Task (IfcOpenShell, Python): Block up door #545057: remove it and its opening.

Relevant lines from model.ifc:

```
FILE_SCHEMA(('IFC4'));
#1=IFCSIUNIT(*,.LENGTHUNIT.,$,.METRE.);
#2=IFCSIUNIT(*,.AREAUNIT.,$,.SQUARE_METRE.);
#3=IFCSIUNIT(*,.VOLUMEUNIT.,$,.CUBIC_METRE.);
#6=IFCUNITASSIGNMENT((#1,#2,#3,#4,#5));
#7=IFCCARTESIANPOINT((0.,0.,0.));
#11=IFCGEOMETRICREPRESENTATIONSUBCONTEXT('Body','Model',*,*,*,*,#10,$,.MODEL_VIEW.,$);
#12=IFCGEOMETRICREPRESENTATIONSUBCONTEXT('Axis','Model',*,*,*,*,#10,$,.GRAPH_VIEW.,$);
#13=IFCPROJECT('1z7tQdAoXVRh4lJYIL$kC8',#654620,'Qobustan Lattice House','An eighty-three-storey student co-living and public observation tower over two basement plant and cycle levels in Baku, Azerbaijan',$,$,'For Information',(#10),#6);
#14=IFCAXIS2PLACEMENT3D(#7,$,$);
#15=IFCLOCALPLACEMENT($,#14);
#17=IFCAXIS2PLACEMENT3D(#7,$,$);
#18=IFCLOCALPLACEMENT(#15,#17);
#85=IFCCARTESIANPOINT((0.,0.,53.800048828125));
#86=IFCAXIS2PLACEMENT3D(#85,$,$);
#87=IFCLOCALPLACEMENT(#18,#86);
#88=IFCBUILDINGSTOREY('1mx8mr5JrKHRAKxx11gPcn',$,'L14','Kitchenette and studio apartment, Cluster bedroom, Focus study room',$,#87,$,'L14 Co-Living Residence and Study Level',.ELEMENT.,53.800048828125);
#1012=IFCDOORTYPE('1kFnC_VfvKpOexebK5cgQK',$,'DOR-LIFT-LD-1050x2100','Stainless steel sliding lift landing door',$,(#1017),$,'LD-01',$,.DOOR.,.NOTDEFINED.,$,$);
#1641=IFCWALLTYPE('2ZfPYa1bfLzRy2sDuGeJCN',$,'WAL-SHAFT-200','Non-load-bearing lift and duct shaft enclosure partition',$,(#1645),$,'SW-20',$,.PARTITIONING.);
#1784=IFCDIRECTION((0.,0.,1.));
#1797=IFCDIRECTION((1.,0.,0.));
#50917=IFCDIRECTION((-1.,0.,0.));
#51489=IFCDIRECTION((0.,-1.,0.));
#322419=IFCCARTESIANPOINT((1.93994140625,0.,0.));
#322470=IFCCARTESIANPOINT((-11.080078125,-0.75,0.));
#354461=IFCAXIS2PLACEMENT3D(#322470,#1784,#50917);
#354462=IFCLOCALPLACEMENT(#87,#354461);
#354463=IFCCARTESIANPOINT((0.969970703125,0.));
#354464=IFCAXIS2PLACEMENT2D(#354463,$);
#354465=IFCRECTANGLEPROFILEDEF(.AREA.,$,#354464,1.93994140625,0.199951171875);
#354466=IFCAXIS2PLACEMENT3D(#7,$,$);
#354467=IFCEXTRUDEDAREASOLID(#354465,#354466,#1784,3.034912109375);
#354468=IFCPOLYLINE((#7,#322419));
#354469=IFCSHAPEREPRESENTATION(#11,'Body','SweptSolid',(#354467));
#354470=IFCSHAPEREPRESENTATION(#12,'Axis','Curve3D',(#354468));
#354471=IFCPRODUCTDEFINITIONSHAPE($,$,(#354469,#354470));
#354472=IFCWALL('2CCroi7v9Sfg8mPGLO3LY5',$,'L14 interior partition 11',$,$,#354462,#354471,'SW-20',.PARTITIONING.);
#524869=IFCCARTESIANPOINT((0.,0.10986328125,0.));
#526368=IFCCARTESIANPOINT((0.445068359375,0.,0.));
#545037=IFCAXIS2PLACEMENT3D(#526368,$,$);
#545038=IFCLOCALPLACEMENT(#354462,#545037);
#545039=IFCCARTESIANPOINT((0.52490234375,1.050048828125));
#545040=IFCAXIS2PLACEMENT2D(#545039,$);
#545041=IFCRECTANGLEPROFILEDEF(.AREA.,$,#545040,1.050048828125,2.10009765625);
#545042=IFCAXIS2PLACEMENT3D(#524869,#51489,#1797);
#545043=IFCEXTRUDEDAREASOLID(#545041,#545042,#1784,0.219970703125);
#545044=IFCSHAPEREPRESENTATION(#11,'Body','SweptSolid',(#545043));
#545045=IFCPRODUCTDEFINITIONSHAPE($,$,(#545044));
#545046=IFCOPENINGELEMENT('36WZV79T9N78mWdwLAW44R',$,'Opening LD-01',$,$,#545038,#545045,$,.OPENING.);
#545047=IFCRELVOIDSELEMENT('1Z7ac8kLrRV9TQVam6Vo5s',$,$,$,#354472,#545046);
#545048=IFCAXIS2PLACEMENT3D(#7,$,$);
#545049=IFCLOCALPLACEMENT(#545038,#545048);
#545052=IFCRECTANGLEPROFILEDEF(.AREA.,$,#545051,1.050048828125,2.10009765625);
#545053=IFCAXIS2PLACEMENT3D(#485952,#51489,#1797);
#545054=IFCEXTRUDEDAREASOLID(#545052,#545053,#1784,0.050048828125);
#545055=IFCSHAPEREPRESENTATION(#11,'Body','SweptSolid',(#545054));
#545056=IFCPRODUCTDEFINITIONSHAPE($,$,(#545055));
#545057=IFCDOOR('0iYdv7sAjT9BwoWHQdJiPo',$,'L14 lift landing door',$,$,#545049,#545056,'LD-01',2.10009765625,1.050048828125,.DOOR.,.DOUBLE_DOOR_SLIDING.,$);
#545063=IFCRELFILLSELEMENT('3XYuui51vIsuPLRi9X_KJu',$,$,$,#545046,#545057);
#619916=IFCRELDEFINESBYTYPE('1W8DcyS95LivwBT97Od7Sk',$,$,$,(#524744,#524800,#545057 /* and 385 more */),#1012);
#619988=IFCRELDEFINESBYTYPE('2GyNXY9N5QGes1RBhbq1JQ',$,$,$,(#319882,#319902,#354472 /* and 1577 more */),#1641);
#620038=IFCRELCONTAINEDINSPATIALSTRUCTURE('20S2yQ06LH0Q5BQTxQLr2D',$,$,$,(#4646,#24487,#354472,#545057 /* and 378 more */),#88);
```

```python
import ifcopenshell
import ifcopenshell.api.feature
import ifcopenshell.api.root
import ifcopenshell.geom
import ifcopenshell.util.shape

model = ifcopenshell.open("model.ifc")
settings = ifcopenshell.geom.settings()


def volume(element):
    """Net volume in cubic metres, openings subtracted."""
    shape = ifcopenshell.geom.create_shape(settings, element)
    return ifcopenshell.util.shape.get_volume(shape.geometry)


door = model.by_guid("0iYdv7sAjT9BwoWHQdJiPo")
opening = door.FillsVoids[0].RelatingOpeningElement
wall = opening.VoidsElements[0].RelatingBuildingElement
before = volume(wall)

ifcopenshell.api.root.remove_product(model, product=door)
ifcopenshell.api.feature.remove_feature(model, feature=opening)

after = volume(wall)

print(f"wall volume {before:.3f} -> {after:.3f} m3")

model.write("model_edited.ifc")
```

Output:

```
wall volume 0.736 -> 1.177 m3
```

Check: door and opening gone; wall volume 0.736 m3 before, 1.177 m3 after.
